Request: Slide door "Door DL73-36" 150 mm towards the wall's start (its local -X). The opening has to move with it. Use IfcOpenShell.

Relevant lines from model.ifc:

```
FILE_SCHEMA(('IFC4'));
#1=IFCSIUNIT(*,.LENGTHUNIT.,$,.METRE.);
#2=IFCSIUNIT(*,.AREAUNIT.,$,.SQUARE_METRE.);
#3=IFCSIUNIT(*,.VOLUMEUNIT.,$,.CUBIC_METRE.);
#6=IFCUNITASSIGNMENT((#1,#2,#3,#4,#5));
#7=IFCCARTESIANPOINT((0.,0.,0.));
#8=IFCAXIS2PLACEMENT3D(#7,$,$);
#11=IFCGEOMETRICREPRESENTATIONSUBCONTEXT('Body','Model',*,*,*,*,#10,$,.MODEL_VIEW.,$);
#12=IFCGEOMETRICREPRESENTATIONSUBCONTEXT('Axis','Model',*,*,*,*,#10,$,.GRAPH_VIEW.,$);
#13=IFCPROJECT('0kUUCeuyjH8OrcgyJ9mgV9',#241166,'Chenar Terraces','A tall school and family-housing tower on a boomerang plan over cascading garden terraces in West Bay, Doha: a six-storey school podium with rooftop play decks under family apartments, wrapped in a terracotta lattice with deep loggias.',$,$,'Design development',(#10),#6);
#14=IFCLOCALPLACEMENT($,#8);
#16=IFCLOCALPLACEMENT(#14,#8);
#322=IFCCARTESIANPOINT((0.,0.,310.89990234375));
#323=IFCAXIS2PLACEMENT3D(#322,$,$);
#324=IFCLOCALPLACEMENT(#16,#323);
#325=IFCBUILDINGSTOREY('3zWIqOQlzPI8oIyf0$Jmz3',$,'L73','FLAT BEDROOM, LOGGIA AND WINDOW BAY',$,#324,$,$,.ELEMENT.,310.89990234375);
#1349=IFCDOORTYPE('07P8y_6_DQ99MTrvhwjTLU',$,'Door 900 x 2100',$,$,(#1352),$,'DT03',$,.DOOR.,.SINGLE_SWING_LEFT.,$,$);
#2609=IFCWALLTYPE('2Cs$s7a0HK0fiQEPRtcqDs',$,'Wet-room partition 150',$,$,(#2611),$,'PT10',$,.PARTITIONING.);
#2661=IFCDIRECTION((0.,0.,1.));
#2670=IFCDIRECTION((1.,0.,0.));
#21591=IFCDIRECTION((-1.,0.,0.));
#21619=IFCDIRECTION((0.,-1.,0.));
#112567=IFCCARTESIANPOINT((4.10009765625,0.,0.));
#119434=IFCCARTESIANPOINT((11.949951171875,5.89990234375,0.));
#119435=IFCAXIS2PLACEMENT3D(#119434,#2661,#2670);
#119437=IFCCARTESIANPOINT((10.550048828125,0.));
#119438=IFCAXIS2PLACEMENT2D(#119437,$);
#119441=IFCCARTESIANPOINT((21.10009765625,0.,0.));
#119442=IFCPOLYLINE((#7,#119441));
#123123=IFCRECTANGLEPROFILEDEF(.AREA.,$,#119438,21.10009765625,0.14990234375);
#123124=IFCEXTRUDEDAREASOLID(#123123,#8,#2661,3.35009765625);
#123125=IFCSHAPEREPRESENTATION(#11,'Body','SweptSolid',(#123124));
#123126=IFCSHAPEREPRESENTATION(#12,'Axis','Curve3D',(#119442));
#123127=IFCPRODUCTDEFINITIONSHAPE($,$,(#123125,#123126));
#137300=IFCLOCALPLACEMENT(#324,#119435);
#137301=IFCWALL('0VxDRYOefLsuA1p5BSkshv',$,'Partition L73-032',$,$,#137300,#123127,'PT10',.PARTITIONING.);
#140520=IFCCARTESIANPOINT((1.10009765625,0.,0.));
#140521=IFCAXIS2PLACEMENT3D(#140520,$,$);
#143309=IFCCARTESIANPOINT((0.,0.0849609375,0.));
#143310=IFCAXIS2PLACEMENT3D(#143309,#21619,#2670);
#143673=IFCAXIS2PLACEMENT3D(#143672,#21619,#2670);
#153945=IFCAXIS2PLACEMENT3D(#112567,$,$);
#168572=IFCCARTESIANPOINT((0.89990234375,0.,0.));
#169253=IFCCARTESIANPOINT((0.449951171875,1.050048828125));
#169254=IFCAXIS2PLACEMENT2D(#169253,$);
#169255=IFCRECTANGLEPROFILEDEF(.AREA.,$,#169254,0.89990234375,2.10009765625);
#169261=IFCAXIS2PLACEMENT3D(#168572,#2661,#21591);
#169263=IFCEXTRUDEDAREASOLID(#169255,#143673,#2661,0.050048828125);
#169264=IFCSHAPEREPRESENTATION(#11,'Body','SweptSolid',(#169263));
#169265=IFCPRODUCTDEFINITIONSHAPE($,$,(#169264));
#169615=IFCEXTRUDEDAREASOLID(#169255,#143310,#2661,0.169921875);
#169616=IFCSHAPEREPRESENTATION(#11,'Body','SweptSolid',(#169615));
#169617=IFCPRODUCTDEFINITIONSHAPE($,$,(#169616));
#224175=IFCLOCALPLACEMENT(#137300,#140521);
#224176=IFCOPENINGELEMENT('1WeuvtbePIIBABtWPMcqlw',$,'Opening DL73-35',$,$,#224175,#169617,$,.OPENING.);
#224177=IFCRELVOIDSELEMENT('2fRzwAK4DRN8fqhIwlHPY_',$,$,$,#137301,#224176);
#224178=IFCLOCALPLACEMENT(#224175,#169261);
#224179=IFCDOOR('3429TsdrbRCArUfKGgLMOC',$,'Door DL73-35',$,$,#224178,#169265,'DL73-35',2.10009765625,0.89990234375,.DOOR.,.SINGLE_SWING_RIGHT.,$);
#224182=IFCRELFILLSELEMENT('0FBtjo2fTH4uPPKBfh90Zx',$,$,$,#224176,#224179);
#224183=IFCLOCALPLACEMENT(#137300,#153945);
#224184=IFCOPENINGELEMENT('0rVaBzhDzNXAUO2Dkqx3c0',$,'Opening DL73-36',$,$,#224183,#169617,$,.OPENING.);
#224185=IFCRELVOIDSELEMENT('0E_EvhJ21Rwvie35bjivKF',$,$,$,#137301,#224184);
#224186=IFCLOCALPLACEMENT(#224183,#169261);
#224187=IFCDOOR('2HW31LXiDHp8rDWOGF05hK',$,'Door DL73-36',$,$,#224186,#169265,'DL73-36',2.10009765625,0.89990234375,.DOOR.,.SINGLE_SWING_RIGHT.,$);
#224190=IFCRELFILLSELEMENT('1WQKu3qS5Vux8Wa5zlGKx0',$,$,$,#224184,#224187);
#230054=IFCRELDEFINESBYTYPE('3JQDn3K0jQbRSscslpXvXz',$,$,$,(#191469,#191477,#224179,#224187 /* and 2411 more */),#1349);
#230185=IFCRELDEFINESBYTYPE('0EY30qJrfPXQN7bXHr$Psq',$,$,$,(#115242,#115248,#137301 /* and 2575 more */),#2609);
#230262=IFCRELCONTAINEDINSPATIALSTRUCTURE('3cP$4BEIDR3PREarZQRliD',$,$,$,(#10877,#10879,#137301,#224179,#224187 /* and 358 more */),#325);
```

```python
import ifcopenshell
import ifcopenshell.api.geometry
import ifcopenshell.util.placement
import ifcopenshell.util.unit

model = ifcopenshell.open("model.ifc")
unit_scale = ifcopenshell.util.unit.calculate_unit_scale(model)

door = model.by_guid("2HW31LXiDHp8rDWOGF05hK")
opening = door.FillsVoids[0].RelatingOpeningElement
wall = opening.VoidsElements[0].RelatingBuildingElement

wall_matrix = ifcopenshell.util.placement.get_local_placement(wall.ObjectPlacement)
shift = wall_matrix[:3, 0] * -0.15 / unit_scale
before = ifcopenshell.util.placement.get_local_placement(door.ObjectPlacement)[:3, 3].copy()

# The door is placed relative to its opening, so it follows when the opening moves.
matrix = ifcopenshell.util.placement.get_local_placement(opening.ObjectPlacement)
matrix[:3, 3] += shift
ifcopenshell.api.geometry.edit_object_placement(
    model, product=opening, matrix=matrix, is_si=False, should_transform_children=True
)

after = ifcopenshell.util.placement.get_local_placement(door.ObjectPlacement)[:3, 3]
print("door moved by", (after - before).round(3) + 0.0)

model.write("model_rev.ifc")
```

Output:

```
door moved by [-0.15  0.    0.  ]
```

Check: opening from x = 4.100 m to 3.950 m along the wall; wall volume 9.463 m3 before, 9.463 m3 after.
